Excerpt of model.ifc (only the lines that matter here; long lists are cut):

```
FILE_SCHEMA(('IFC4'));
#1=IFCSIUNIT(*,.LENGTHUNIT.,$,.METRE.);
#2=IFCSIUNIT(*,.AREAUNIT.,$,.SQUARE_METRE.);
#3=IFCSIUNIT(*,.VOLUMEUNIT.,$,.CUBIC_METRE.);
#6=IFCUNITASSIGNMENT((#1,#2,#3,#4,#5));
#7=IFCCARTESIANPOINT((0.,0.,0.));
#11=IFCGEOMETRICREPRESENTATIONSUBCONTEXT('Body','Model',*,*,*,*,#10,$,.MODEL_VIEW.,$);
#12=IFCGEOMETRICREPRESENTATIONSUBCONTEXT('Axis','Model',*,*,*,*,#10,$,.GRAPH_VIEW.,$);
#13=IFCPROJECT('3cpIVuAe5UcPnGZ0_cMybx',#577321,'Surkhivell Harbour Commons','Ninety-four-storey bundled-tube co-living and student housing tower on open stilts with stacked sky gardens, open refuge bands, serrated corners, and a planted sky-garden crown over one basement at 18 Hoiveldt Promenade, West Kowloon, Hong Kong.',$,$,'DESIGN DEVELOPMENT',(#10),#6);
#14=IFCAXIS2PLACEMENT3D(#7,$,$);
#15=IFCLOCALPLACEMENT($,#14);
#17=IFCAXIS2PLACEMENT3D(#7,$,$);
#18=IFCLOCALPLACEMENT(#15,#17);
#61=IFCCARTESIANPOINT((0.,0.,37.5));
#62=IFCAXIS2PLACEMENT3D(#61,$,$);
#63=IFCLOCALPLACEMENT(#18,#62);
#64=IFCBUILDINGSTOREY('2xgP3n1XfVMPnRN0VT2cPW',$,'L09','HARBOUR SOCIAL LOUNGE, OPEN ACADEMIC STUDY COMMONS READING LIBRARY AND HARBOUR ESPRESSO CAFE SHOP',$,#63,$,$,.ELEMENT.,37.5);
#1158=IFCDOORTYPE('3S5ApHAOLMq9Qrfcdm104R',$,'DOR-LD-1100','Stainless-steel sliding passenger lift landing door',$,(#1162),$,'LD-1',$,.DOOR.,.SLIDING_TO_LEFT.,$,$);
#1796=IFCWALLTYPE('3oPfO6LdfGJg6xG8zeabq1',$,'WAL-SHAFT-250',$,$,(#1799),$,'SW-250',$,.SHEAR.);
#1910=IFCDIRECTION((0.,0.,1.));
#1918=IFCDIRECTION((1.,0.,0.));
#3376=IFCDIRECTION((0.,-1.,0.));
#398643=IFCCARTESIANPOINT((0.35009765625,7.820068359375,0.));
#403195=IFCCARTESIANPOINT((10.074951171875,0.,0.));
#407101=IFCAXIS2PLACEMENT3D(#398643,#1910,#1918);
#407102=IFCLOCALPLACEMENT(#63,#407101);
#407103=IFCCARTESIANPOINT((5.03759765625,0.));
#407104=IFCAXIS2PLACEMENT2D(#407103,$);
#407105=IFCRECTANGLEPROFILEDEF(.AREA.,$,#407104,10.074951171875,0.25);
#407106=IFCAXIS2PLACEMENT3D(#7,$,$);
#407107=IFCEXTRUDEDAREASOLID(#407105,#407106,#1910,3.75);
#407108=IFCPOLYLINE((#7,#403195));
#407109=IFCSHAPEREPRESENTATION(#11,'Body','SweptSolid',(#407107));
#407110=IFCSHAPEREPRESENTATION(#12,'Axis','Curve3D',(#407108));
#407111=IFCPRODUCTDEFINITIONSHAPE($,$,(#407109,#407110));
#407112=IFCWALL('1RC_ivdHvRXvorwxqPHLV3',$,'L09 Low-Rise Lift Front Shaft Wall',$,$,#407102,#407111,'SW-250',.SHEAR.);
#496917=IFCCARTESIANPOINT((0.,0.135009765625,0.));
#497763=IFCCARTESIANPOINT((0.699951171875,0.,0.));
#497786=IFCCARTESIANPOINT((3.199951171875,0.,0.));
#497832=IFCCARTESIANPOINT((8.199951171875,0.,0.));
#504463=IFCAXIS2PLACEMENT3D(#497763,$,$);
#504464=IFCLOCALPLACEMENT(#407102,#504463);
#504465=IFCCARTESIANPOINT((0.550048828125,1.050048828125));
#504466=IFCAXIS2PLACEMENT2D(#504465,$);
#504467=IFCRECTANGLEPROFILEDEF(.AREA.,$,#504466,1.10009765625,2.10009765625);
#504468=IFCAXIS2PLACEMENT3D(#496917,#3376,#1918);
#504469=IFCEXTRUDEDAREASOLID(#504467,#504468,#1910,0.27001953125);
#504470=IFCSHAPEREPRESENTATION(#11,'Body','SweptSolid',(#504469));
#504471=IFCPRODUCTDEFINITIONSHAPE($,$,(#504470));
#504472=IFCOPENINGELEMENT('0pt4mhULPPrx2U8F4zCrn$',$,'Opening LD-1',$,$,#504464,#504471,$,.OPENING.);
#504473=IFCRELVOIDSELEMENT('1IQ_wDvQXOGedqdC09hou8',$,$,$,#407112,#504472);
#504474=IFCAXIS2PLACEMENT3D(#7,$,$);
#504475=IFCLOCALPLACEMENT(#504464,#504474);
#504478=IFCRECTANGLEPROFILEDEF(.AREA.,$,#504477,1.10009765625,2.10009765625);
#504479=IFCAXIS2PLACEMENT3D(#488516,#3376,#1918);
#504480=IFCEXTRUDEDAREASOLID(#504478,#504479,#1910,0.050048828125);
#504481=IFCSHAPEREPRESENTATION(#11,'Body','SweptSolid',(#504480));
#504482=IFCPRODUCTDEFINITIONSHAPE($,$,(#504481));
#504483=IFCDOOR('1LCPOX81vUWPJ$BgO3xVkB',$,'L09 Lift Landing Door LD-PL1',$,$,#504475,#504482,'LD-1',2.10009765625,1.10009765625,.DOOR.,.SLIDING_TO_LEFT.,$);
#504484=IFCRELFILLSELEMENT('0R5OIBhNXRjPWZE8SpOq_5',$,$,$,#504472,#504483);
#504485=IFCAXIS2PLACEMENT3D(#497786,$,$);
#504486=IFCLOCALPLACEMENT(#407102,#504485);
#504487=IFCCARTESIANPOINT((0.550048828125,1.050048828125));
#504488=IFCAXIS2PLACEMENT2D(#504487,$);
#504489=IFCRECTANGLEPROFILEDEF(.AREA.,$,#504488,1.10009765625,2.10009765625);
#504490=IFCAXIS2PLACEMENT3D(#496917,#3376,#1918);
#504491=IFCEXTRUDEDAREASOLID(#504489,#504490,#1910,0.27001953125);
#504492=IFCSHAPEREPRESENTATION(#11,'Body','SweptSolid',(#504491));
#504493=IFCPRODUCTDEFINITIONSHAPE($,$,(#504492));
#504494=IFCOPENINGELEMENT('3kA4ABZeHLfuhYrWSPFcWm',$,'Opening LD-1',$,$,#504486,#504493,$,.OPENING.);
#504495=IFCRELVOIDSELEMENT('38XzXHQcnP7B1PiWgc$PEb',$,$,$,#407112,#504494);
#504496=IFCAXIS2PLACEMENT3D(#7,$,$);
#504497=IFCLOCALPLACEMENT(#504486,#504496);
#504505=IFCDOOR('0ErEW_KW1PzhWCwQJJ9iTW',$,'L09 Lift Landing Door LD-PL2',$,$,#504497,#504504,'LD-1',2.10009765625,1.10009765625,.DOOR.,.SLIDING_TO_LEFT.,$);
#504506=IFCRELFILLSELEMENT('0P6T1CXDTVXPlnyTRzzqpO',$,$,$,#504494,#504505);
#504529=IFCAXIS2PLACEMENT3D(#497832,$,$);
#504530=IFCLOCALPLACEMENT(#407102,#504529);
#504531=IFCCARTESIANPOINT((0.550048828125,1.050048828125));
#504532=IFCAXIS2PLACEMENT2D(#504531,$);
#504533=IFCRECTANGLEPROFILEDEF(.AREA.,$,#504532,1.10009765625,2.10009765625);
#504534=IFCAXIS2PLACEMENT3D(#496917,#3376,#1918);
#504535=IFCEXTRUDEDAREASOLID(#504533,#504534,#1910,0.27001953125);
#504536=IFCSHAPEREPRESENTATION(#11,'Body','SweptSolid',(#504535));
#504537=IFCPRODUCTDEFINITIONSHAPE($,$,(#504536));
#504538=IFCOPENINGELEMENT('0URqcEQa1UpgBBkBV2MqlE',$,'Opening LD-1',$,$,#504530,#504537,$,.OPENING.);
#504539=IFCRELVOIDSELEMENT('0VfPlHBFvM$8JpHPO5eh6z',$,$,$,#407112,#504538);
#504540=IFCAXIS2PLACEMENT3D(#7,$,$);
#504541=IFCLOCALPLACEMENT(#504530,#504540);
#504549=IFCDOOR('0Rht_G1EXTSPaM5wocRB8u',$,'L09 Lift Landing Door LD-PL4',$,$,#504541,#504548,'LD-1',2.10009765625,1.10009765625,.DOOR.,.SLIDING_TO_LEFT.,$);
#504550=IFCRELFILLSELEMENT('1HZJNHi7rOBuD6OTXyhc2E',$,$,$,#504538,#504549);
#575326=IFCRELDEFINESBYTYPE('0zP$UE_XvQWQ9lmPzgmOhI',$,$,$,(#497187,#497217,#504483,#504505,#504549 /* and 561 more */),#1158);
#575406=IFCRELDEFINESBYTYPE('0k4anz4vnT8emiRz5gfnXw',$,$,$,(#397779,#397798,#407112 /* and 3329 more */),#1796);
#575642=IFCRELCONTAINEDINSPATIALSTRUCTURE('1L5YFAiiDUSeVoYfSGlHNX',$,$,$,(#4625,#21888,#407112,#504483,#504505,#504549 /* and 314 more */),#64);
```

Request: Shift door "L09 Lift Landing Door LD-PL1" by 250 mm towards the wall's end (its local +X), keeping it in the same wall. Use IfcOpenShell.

```python
import ifcopenshell
import ifcopenshell.api.geometry
import ifcopenshell.util.placement
import ifcopenshell.util.unit

model = ifcopenshell.open("model.ifc")
unit_scale = ifcopenshell.util.unit.calculate_unit_scale(model)

door = model.by_guid("1LCPOX81vUWPJ$BgO3xVkB")
opening = door.FillsVoids[0].RelatingOpeningElement
wall = opening.VoidsElements[0].RelatingBuildingElement

wall_matrix = ifcopenshell.util.placement.get_local_placement(wall.ObjectPlacement)
shift = wall_matrix[:3, 0] * 0.25 / unit_scale
before = ifcopenshell.util.placement.get_local_placement(door.ObjectPlacement)[:3, 3].copy()

# The door is placed relative to its opening, so it follows when the opening moves.
matrix = ifcopenshell.util.placement.get_local_placement(opening.ObjectPlacement)
matrix[:3, 3] += shift
ifcopenshell.api.geometry.edit_object_placement(
    model, product=opening, matrix=matrix, is_si=False, should_transform_children=True
)

after = ifcopenshell.util.placement.get_local_placement(door.ObjectPlacement)[:3, 3]
print("door moved by", (after - before).round(3) + 0.0)

model.write("model-out.ifc")
```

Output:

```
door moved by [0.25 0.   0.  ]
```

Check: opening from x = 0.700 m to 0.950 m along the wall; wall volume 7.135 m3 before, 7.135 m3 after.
